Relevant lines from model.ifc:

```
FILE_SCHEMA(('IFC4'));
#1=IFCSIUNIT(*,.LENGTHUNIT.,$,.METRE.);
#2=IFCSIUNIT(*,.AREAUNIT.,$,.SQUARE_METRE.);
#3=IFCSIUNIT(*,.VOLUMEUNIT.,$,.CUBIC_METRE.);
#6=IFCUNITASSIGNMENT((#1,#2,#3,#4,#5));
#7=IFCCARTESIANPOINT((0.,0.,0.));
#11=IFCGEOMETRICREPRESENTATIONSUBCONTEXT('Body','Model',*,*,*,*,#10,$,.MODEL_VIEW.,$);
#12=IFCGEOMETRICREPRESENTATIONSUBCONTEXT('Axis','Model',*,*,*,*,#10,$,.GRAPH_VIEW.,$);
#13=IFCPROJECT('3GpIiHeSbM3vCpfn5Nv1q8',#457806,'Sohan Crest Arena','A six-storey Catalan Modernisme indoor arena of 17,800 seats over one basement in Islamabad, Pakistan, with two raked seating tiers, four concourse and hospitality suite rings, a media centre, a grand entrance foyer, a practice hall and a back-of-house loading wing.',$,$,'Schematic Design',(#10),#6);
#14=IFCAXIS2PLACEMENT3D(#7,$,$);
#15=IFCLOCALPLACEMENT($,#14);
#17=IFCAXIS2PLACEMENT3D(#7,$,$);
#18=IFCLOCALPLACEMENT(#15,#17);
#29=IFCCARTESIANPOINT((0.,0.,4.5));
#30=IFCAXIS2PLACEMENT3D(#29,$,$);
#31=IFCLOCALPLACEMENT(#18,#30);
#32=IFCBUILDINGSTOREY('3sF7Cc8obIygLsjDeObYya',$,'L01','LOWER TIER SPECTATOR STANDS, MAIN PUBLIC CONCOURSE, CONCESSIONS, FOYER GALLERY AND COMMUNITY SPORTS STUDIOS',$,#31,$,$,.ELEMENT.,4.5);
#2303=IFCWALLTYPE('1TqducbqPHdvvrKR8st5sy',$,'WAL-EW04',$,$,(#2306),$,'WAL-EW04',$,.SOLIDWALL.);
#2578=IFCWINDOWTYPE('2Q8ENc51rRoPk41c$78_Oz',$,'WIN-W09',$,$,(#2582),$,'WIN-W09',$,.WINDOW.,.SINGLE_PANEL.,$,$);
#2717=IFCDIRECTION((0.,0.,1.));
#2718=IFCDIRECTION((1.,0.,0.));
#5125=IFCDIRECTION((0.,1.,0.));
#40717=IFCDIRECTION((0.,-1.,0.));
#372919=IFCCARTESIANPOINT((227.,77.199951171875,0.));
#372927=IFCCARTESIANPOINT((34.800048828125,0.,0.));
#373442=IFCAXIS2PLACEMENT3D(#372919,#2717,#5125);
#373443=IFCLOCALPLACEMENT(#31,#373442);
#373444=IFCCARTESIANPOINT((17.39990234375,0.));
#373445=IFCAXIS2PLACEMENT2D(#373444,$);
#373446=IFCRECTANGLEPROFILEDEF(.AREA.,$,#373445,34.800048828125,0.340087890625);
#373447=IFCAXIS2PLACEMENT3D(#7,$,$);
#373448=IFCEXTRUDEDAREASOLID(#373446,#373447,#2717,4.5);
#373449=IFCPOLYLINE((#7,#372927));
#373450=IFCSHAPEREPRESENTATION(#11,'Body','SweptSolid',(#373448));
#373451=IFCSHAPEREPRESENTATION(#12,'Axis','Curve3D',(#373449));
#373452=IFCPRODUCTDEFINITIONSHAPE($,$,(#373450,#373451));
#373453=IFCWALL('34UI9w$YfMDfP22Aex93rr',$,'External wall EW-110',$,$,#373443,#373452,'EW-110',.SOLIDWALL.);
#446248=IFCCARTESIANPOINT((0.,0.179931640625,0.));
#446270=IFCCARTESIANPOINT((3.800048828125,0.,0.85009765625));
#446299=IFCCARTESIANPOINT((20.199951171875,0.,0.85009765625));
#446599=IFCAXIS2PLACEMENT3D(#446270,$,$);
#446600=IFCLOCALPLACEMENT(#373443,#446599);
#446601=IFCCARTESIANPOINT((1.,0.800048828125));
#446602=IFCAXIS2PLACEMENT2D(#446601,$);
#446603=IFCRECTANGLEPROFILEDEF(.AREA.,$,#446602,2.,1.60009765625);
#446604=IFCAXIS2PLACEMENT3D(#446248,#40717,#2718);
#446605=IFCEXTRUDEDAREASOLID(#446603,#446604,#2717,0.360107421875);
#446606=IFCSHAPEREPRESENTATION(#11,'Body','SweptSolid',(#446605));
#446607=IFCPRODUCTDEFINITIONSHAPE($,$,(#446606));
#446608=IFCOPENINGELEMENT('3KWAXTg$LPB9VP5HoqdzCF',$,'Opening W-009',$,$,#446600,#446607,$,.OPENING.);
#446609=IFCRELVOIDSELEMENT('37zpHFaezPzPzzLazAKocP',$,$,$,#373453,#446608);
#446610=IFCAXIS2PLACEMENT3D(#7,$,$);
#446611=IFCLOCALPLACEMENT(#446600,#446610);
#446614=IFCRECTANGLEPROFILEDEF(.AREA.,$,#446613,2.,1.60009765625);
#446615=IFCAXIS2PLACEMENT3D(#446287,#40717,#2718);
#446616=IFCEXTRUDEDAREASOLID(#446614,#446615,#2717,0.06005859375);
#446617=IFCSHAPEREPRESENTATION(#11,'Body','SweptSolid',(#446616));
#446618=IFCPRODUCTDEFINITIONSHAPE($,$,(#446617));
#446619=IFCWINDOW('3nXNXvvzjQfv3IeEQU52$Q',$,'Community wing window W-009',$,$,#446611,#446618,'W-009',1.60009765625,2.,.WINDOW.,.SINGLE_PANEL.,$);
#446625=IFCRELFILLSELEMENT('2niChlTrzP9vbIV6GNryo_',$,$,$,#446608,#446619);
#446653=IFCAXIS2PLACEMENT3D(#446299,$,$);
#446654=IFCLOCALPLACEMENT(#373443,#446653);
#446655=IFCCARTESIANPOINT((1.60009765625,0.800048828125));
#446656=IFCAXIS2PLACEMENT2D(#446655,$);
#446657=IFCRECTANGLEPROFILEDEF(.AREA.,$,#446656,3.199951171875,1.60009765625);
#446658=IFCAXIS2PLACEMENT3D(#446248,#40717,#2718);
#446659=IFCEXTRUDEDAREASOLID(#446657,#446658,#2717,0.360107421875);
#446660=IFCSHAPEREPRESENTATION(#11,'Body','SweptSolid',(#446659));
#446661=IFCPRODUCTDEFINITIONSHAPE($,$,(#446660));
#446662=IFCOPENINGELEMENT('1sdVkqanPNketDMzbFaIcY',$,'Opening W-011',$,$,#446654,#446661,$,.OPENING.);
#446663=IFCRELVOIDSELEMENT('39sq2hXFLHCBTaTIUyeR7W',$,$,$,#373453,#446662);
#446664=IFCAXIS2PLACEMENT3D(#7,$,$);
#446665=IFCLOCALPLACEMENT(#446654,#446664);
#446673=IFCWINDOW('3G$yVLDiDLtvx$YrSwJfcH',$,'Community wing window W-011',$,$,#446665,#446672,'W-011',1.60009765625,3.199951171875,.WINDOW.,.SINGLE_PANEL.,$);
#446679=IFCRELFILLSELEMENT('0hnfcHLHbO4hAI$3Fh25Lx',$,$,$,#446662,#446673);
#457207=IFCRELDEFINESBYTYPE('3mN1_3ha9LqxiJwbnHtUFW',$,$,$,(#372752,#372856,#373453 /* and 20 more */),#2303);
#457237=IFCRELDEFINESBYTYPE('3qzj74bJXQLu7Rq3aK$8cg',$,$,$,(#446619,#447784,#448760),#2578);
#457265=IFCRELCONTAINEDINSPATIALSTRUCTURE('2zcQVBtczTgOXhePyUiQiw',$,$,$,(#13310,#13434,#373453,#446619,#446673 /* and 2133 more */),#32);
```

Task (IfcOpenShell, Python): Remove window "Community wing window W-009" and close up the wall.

```python
import ifcopenshell
import ifcopenshell.api.feature
import ifcopenshell.api.root
import ifcopenshell.geom
import ifcopenshell.util.shape

model = ifcopenshell.open("model.ifc")
settings = ifcopenshell.geom.settings()


def volume(element):
    """Net volume in cubic metres, openings subtracted."""
    shape = ifcopenshell.geom.create_shape(settings, element)
    return ifcopenshell.util.shape.get_volume(shape.geometry)


window = model.by_guid("3nXNXvvzjQfv3IeEQU52$Q")
opening = window.FillsVoids[0].RelatingOpeningElement
wall = opening.VoidsElements[0].RelatingBuildingElement
before = volume(wall)

ifcopenshell.api.root.remove_product(model, product=window)
ifcopenshell.api.feature.remove_feature(model, feature=opening)

after = volume(wall)

print(f"wall volume {before:.3f} -> {after:.3f} m3")

model.write("model-out.ifc")
```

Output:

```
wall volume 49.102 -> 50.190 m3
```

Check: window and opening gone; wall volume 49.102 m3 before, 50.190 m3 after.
